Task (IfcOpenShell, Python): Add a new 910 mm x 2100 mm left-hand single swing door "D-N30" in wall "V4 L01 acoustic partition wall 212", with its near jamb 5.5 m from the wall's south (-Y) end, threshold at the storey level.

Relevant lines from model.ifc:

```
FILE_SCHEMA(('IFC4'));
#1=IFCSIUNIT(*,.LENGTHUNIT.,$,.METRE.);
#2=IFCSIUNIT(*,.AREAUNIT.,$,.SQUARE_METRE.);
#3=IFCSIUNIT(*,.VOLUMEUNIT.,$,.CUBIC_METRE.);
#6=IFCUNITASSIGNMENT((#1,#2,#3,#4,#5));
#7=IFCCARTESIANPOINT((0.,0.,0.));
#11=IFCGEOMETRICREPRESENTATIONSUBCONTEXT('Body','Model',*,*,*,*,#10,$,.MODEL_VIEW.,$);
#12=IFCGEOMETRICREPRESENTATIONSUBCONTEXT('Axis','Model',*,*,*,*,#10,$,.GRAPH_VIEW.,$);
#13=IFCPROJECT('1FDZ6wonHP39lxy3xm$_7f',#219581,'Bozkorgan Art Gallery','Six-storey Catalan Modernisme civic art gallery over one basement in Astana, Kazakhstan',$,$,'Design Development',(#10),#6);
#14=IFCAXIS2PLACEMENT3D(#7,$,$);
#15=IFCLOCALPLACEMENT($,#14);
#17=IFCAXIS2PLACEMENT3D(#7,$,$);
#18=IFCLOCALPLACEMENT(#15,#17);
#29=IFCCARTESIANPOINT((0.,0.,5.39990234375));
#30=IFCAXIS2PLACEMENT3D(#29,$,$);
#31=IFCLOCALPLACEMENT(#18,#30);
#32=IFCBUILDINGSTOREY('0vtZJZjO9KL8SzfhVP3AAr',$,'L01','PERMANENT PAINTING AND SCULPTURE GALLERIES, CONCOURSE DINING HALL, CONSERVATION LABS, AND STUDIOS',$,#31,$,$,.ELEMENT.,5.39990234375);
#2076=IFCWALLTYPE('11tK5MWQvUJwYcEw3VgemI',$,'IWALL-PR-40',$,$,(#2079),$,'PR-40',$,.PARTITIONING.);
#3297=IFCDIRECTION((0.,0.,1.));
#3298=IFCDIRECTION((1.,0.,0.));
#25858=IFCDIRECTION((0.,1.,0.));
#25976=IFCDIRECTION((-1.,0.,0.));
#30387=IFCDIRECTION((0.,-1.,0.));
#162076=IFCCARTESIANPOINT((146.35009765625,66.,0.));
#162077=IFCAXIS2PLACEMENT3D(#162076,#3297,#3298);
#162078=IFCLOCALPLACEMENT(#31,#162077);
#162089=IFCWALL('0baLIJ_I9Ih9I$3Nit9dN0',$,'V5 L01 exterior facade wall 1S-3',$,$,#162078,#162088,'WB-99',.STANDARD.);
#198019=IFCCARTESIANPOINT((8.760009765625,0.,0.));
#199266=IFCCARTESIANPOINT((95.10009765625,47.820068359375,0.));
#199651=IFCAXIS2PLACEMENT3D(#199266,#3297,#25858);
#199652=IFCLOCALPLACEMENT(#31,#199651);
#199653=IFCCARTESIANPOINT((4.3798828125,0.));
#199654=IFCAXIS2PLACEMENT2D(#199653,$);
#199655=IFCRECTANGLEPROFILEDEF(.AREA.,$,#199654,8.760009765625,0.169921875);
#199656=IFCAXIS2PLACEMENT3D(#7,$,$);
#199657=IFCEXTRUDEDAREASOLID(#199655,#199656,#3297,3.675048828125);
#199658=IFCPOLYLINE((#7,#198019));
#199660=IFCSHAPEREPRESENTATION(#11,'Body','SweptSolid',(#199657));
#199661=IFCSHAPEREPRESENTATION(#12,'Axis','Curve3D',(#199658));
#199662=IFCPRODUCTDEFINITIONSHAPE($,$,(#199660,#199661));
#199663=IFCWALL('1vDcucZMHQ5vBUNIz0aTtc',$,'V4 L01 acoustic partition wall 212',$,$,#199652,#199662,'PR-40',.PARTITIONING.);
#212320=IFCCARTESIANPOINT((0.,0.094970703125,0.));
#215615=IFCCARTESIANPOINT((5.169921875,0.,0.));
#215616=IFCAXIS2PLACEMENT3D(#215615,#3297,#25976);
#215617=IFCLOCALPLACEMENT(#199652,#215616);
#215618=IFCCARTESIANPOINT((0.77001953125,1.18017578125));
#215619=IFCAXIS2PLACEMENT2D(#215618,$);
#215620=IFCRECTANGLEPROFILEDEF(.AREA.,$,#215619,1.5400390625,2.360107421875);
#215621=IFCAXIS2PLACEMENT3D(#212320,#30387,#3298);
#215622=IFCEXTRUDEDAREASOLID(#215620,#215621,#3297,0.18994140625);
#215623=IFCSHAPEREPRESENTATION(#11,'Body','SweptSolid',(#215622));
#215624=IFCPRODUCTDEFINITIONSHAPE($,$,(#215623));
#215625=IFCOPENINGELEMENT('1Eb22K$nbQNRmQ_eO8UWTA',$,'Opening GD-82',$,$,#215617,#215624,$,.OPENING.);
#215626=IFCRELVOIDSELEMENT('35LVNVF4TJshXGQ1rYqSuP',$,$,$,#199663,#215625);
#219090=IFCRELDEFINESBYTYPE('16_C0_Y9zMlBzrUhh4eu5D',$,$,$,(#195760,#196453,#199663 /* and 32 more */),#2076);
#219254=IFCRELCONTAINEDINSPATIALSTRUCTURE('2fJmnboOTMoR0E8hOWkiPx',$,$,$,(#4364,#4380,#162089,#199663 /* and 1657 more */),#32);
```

```python
import numpy as np
import ifcopenshell
import ifcopenshell.api.feature
import ifcopenshell.api.geometry
import ifcopenshell.api.root
import ifcopenshell.api.spatial
import ifcopenshell.geom
import ifcopenshell.util.element
import ifcopenshell.util.placement
import ifcopenshell.util.representation
import ifcopenshell.util.shape
import ifcopenshell.util.unit

model = ifcopenshell.open("model.ifc")
unit_scale = ifcopenshell.util.unit.calculate_unit_scale(model)
settings = ifcopenshell.geom.settings()


def volume(element):
    """Net volume in cubic metres, openings subtracted."""
    shape = ifcopenshell.geom.create_shape(settings, element)
    return ifcopenshell.util.shape.get_volume(shape.geometry)


wall = model.by_guid("1vDcucZMHQ5vBUNIz0aTtc")
storey = ifcopenshell.util.element.get_container(wall, ifc_class="IfcBuildingStorey")
context = ifcopenshell.util.representation.get_context(model, "Model", "Body", "MODEL_VIEW")
before = volume(wall)

width, height, from_end, sill = 0.91, 2.1, 5.5, 0.0  # metres

# The wall runs along its own X axis, and the end named is its -X end.
wall_shape = ifcopenshell.geom.create_shape(settings, wall)
x, y, z = ifcopenshell.util.shape.get_vertices(wall_shape.geometry).T
start = x.min() + from_end
face, thickness = float(y.min()), float(y.max() - y.min())
wall_matrix = ifcopenshell.util.placement.get_local_placement(wall.ObjectPlacement)
level = ifcopenshell.util.placement.get_local_placement(storey.ObjectPlacement)[2, 3]


def in_wall(x, y):
    """Placement at x, y metres in the wall's axes, at sill height."""
    matrix = wall_matrix.copy()
    matrix[:, 3] = wall_matrix @ np.array([x / unit_scale, y / unit_scale, 0.0, 1.0])
    matrix[2, 3] = level + sill / unit_scale
    return matrix


# Opening: a box that overshoots both wall faces by 50 mm.
opening = ifcopenshell.api.root.create_entity(model, ifc_class="IfcOpeningElement", predefined_type="OPENING")
box = ifcopenshell.api.geometry.add_wall_representation(
    model, context=context, length=width, height=height, thickness=thickness + 0.1
)
ifcopenshell.api.geometry.assign_representation(model, product=opening, representation=box)
ifcopenshell.api.geometry.edit_object_placement(model, product=opening, matrix=in_wall(start, face - 0.05), is_si=False)
ifcopenshell.api.feature.add_feature(model, feature=opening, element=wall)

door = ifcopenshell.api.root.create_entity(model, ifc_class="IfcDoor", name="D-N30", predefined_type="DOOR")
door.OverallWidth, door.OverallHeight = width / unit_scale, height / unit_scale
door.OperationType = "SINGLE_SWING_LEFT"
body = ifcopenshell.api.geometry.add_door_representation(
    model,
    context=context,
    overall_width=door.OverallWidth,
    overall_height=door.OverallHeight,
    operation_type="SINGLE_SWING_LEFT",
    lining_properties={"LiningDepth": thickness / unit_scale, "ThresholdDepth": thickness / unit_scale},
)
ifcopenshell.api.geometry.assign_representation(model, product=door, representation=body)
ifcopenshell.api.spatial.assign_container(model, products=[door], relating_structure=storey)
ifcopenshell.api.feature.add_filling(model, opening=opening, element=door)

# The lining spans the wall, so the door starts at the wall face.
ifcopenshell.api.geometry.edit_object_placement(model, product=door, matrix=in_wall(start, face), is_si=False)

after = volume(wall)

print(f"wall volume {before:.3f} -> {after:.3f} m3")

model.write("model_v2.ifc")
```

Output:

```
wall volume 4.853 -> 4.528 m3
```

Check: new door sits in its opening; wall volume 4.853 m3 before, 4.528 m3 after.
